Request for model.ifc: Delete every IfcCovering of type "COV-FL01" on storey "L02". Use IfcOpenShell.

First a look at what the model holds.

```python
import ifcopenshell
import ifcopenshell.util.element

model = ifcopenshell.open("model.ifc")
print(model.schema)
storey = next(s for s in model.by_type("IfcBuildingStorey") if s.Name == "L02")
coverings = [e for e in ifcopenshell.util.element.get_decomposition(storey) if e.is_a("IfcCovering")]
seen = {}
for e in coverings:
    element_type = ifcopenshell.util.element.get_type(e)
    name = element_type.Name if element_type not in (None, e) else None
    seen[name] = seen.get(name, 0) + 1
for name, count in sorted(seen.items(), key=str):
    print(count, "x", name)
```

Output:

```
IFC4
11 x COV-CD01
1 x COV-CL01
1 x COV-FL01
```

```python
import ifcopenshell
import ifcopenshell.api.root
import ifcopenshell.util.element

model = ifcopenshell.open("model.ifc")

storey = next(s for s in model.by_type("IfcBuildingStorey") if s.Name == "L02")
coverings = [e for e in ifcopenshell.util.element.get_decomposition(storey) if e.is_a("IfcCovering")]
targets = [e for e in coverings if (t := ifcopenshell.util.element.get_type(e)) not in (None, e) and t.Name == "COV-FL01"]

for e in targets:
    ifcopenshell.api.root.remove_product(model, product=e)
print(len(targets), "removed")

model.write("model_rev.ifc")
```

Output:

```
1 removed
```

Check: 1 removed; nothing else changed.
